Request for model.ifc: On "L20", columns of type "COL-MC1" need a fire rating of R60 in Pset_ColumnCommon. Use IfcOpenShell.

First a look at what the model holds.

```python
import ifcopenshell
import ifcopenshell.util.element

model = ifcopenshell.open("model.ifc")
print(model.schema)
storey = next(s for s in model.by_type("IfcBuildingStorey") if s.Name == "L20")
columns = [e for e in ifcopenshell.util.element.get_decomposition(storey) if e.is_a("IfcColumn")]
seen = {}
for e in columns:
    element_type = ifcopenshell.util.element.get_type(e)
    key = (element_type.Name if element_type != e and element_type else None, ifcopenshell.util.element.get_pset(e, "Pset_ColumnCommon", "FireRating"))
    seen[key] = seen.get(key, 0) + 1
for (name, value), count in sorted(seen.items(), key=str):
    print(count, "x", name, "|", value)
```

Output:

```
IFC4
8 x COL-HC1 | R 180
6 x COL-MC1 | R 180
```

```python
import ifcopenshell
import ifcopenshell.api.pset
import ifcopenshell.util.element

model = ifcopenshell.open("model.ifc")

storey = next(s for s in model.by_type("IfcBuildingStorey") if s.Name == "L20")
columns = [e for e in ifcopenshell.util.element.get_decomposition(storey) if e.is_a("IfcColumn")]

count = 0
for e in columns:
    element_type = ifcopenshell.util.element.get_type(e)
    if element_type in (None, e) or element_type.Name != "COL-MC1":
        continue
    found = ifcopenshell.util.element.get_pset(e, "Pset_ColumnCommon", should_inherit=False)
    if found:
        pset = model.by_id(found["id"])
        if len(ifcopenshell.util.element.get_elements_by_pset(pset)) > 1:
            pset = ifcopenshell.api.pset.unshare_pset(model, products=[e], pset=pset)[0]
    else:
        pset = ifcopenshell.api.pset.add_pset(model, product=e, name="Pset_ColumnCommon")
    ifcopenshell.api.pset.edit_pset(model, pset=pset, properties={"FireRating": "R60"})
    count += 1

print(count, "columns updated")

model.write("model-out.ifc")
```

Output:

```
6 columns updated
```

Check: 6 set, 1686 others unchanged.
